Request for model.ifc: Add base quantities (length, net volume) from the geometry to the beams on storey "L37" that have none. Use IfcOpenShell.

First a look at what the model holds.

```python
import ifcopenshell
import ifcopenshell.util.element
import ifcopenshell.util.unit

model = ifcopenshell.open("model.ifc")
print(model.schema)
for unit_type in ("LENGTHUNIT", "AREAUNIT", "VOLUMEUNIT"):
    print(unit_type, ifcopenshell.util.unit.calculate_unit_scale(model, unit_type))
storey = next(s for s in model.by_type("IfcBuildingStorey") if s.Name == "L37")
beams = [e for e in ifcopenshell.util.element.get_decomposition(storey) if e.is_a("IfcBeam")]
for e in sorted(beams, key=lambda e: e.id()):
    print(e.id(), e.is_a(), e.Name, list(ifcopenshell.util.element.get_psets(e, qtos_only=True)), sep=" | ")
```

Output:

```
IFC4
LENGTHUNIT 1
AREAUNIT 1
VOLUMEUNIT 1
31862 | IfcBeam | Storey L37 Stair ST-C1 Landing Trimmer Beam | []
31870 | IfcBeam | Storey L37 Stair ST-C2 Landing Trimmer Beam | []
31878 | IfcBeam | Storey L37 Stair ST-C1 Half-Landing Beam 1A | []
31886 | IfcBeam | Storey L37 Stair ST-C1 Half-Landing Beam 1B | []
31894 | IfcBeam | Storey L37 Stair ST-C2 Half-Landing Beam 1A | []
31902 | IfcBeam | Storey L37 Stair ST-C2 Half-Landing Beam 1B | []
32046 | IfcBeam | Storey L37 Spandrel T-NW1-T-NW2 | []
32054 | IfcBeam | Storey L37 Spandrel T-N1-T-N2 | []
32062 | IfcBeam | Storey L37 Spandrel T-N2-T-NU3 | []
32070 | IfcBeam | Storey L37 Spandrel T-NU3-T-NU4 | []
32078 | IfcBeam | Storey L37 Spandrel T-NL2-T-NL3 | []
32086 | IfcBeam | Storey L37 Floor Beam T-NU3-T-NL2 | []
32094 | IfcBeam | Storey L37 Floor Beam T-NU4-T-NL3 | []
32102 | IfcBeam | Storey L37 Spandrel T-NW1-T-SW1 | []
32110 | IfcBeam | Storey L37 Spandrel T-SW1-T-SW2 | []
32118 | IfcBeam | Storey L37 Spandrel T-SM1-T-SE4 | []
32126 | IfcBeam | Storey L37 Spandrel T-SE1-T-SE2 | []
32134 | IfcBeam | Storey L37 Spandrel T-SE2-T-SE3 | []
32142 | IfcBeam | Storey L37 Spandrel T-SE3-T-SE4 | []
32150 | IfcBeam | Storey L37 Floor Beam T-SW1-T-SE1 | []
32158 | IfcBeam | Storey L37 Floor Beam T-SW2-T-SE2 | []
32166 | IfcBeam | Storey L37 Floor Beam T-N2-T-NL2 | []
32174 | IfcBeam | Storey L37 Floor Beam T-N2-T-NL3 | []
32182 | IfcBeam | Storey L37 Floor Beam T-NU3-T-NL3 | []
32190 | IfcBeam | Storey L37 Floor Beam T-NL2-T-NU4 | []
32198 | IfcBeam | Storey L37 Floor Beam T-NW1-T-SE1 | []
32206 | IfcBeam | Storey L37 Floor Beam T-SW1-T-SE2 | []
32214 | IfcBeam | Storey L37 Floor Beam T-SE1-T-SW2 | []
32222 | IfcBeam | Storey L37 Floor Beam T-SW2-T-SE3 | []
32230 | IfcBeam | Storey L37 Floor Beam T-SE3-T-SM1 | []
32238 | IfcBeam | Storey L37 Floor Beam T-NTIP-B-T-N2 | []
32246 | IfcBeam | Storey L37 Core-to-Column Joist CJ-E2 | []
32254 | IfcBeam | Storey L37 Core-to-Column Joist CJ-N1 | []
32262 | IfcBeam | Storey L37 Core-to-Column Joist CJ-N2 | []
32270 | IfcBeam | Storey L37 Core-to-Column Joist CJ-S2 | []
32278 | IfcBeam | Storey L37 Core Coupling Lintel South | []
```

```python
import ifcopenshell
import ifcopenshell.api.pset
import ifcopenshell.geom
import ifcopenshell.util.element
import ifcopenshell.util.shape
import ifcopenshell.util.unit

model = ifcopenshell.open("model.ifc")
unit_scale = ifcopenshell.util.unit.calculate_unit_scale(model)
volume_scale = ifcopenshell.util.unit.calculate_unit_scale(model, "VOLUMEUNIT")
settings = ifcopenshell.geom.settings()

storey = next(s for s in model.by_type("IfcBuildingStorey") if s.Name == "L37")
beams = [e for e in ifcopenshell.util.element.get_decomposition(storey) if e.is_a("IfcBeam")]

for e in sorted(beams, key=lambda e: e.id()):
    if ifcopenshell.util.element.get_psets(e, qtos_only=True, should_inherit=False):
        continue
    # Geometry comes back in metres, in the element's own axes.
    shape = ifcopenshell.geom.create_shape(settings, e)
    values = {
        "Length": ifcopenshell.util.shape.get_max_xyz(shape.geometry) / unit_scale,
        "NetVolume": ifcopenshell.util.shape.get_volume(shape.geometry) / volume_scale,
    }
    qto = ifcopenshell.api.pset.add_qto(model, product=e, name="Qto_BeamBaseQuantities")
    ifcopenshell.api.pset.edit_qto(model, qto=qto, properties=values)
    print(e.id(), {k: round(v, 3) for k, v in values.items()})

model.write("model-out.ifc")
```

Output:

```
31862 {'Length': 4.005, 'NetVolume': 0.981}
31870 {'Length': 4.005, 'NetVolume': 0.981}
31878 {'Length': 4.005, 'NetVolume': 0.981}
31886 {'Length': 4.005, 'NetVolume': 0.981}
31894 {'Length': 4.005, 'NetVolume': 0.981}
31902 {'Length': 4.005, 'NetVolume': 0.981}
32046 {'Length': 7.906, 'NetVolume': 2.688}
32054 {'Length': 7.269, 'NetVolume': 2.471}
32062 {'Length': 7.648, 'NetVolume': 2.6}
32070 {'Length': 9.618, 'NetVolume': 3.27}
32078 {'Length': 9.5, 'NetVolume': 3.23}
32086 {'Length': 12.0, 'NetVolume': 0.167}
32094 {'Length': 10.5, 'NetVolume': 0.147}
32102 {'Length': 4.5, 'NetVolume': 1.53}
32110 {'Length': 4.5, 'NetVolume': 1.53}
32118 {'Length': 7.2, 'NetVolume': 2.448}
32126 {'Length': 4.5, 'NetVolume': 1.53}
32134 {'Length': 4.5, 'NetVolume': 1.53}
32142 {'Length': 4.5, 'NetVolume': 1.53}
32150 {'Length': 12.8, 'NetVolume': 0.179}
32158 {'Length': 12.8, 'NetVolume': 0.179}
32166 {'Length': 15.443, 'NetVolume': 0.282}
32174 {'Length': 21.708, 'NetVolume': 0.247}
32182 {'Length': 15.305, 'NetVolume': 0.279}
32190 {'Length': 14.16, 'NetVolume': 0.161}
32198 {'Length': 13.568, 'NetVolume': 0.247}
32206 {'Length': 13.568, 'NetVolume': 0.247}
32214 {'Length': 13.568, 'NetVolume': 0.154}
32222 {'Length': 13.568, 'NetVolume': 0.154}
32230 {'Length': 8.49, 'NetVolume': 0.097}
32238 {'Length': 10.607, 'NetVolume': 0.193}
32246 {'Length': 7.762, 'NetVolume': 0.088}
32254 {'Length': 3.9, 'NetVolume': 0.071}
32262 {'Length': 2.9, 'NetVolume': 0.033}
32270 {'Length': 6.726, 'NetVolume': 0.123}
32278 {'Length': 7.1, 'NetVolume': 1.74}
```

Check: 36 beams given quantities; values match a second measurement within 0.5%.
